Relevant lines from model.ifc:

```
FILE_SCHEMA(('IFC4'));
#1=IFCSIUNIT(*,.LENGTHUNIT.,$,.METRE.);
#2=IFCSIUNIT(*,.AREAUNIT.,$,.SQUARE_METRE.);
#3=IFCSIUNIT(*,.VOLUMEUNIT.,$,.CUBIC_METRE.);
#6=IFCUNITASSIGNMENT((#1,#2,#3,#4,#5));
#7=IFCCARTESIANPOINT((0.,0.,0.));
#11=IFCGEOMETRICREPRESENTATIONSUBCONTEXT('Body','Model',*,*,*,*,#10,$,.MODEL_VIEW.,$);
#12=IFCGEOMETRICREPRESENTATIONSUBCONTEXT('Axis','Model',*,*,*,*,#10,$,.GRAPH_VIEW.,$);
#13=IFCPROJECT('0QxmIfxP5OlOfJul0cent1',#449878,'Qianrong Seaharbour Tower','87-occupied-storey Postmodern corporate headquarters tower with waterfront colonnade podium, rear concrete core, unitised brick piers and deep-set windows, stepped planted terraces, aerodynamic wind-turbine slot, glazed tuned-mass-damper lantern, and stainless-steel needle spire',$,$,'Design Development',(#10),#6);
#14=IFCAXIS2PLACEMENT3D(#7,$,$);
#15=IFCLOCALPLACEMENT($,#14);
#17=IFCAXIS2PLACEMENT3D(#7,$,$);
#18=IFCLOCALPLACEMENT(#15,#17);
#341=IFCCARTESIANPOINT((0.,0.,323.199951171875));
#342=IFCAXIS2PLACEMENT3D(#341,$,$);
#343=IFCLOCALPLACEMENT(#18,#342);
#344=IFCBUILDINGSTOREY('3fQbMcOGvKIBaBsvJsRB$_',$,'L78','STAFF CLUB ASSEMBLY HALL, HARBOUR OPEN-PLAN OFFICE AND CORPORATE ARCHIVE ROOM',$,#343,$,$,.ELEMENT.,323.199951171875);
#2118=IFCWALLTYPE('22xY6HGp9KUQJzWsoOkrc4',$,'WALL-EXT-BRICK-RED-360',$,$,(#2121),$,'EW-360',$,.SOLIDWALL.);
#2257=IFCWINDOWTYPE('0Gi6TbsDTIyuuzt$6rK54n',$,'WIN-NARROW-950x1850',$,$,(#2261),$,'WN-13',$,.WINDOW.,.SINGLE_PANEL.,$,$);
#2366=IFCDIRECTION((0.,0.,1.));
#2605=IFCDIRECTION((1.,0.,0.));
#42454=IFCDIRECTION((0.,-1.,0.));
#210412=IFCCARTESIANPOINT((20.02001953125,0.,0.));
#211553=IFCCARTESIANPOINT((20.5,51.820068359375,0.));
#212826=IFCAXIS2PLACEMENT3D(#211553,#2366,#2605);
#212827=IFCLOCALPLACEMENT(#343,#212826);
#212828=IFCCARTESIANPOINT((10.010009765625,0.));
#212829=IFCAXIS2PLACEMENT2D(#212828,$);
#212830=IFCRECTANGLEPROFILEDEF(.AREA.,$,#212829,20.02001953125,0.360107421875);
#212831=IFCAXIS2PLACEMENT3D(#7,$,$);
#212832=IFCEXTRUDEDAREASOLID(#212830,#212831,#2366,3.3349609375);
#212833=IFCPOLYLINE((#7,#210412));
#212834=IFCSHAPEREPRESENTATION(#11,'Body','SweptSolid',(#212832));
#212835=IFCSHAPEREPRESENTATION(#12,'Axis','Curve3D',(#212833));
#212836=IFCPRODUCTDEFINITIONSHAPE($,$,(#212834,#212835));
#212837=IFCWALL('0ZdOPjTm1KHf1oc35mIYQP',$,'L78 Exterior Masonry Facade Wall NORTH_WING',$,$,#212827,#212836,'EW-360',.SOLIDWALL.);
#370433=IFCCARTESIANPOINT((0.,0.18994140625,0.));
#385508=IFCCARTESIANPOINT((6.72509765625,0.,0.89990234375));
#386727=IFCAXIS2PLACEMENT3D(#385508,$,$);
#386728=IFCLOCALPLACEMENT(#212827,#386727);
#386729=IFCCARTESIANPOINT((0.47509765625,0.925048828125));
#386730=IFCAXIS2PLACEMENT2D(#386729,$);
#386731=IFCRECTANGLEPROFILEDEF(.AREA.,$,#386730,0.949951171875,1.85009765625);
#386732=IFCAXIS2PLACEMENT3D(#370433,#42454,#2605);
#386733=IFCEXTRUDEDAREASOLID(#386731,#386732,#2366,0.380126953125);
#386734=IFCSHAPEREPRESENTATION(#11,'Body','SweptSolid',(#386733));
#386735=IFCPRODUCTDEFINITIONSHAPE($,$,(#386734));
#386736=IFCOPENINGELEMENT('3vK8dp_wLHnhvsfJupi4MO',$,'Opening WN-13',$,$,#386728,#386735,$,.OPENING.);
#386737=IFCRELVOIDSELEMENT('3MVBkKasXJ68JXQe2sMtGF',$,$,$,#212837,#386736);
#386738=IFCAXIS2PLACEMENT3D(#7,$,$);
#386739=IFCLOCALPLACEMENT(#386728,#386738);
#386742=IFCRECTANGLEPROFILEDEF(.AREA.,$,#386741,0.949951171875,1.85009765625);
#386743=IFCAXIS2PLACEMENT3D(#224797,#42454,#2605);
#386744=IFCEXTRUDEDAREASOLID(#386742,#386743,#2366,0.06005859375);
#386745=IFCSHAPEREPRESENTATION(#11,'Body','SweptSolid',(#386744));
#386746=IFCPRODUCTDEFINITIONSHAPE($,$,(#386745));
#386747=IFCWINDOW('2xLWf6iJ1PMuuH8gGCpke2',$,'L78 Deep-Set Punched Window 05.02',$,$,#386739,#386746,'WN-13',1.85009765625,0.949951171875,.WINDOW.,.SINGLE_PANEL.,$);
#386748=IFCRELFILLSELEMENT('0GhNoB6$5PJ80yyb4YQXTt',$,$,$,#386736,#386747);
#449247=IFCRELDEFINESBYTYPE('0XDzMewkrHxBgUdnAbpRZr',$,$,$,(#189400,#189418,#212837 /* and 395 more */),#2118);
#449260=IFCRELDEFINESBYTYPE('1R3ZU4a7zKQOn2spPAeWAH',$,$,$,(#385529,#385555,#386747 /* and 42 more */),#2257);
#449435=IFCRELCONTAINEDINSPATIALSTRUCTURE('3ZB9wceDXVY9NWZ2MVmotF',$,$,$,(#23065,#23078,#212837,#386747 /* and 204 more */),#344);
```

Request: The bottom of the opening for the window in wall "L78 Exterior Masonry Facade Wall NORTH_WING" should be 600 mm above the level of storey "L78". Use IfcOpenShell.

```python
import numpy as np
import ifcopenshell
import ifcopenshell.api.geometry
import ifcopenshell.geom
import ifcopenshell.util.element
import ifcopenshell.util.placement
import ifcopenshell.util.shape
import ifcopenshell.util.unit

model = ifcopenshell.open("model.ifc")
unit_scale = ifcopenshell.util.unit.calculate_unit_scale(model)

window = model.by_id(386747)
opening = window.FillsVoids[0].RelatingOpeningElement
storey = ifcopenshell.util.element.get_container(window, ifc_class="IfcBuildingStorey")
level = ifcopenshell.util.placement.get_local_placement(storey.ObjectPlacement)[2, 3]

# The opening's origin need not be at the sill, so measure its lowest point.
shape = ifcopenshell.geom.create_shape(ifcopenshell.geom.settings(), opening)
bottom = ifcopenshell.util.shape.get_shape_bottom_elevation(shape, shape.geometry) / unit_scale
dz = level + 0.6 / unit_scale - bottom

shift = np.array([0.0, 0.0, dz])
# The window is placed relative to its opening, so it follows when the opening moves.
matrix = ifcopenshell.util.placement.get_local_placement(opening.ObjectPlacement)
matrix[:3, 3] += shift
ifcopenshell.api.geometry.edit_object_placement(
    model, product=opening, matrix=matrix, is_si=False, should_transform_children=True
)

print(f"moved by {dz * unit_scale:+.3f} m")

model.write("model_updated.ifc")
```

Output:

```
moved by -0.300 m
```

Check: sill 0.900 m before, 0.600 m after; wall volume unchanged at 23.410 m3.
